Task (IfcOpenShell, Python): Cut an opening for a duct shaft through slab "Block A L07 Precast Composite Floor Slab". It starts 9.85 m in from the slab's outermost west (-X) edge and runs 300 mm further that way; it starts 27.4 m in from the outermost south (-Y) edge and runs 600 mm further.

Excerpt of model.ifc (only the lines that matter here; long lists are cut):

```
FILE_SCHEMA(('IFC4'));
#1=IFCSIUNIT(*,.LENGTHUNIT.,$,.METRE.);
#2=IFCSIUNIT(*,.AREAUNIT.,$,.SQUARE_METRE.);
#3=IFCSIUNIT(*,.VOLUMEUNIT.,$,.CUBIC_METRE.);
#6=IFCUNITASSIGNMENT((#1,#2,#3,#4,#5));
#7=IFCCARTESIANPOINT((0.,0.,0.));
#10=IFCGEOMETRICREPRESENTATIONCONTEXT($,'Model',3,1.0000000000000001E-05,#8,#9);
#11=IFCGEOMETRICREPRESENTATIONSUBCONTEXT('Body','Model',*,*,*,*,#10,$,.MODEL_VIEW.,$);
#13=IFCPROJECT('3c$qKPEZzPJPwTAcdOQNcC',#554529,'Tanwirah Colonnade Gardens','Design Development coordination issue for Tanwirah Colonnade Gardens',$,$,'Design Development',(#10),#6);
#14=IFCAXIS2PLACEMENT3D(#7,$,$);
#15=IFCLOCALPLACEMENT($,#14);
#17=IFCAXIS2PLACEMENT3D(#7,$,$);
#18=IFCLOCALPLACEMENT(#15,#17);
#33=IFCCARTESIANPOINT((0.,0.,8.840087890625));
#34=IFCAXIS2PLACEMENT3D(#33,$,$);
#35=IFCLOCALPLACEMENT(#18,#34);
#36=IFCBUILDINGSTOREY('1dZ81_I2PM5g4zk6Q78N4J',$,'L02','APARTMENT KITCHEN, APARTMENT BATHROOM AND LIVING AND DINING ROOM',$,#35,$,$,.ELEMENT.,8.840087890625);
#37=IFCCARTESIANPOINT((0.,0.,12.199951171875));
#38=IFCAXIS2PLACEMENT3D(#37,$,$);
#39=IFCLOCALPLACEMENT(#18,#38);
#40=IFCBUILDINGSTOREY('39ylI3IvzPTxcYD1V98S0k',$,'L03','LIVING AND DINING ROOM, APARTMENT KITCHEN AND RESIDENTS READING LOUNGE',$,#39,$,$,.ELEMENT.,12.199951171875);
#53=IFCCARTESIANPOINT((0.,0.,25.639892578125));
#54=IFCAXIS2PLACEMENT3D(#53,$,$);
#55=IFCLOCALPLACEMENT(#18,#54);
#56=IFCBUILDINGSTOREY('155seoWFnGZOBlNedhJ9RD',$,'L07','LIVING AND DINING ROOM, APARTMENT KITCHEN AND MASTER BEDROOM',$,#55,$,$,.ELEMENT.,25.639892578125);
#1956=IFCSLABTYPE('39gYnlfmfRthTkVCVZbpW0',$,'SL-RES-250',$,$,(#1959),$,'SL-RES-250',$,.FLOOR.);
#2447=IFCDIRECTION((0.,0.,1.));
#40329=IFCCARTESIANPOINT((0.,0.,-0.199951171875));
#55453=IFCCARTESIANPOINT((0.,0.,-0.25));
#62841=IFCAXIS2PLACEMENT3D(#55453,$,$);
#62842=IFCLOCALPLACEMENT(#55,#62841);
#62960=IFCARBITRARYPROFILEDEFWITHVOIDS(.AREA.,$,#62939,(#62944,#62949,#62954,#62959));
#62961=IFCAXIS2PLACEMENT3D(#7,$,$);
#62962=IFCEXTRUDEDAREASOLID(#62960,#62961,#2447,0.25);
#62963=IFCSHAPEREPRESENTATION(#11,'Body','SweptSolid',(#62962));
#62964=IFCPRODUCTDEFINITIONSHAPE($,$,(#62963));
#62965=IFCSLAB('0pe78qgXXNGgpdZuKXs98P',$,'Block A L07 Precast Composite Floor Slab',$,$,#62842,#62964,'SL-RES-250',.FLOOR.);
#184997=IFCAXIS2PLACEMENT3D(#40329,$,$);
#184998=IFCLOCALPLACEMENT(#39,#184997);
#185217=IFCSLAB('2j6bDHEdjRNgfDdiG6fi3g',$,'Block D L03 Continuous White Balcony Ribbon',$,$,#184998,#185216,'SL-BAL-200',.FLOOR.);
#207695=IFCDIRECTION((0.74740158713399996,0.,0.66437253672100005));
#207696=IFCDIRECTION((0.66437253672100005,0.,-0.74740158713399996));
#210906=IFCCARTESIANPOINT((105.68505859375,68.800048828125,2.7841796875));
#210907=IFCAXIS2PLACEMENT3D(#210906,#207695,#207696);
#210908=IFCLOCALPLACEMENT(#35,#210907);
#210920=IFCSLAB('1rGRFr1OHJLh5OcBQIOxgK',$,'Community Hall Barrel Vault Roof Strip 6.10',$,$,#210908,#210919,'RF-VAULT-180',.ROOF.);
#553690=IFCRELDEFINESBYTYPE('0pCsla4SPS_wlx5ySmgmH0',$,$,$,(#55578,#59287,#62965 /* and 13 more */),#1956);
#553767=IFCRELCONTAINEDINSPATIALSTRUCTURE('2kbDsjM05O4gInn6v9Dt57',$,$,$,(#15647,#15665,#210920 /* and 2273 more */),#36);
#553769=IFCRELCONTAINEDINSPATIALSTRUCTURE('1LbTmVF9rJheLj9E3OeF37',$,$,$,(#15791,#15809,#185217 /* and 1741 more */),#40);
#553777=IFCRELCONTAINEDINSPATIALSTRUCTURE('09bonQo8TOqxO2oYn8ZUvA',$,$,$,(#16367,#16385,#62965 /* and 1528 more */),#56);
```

```python
import numpy as np
import ifcopenshell
import ifcopenshell.api.feature
import ifcopenshell.api.geometry
import ifcopenshell.api.root
import ifcopenshell.geom
import ifcopenshell.util.placement
import ifcopenshell.util.representation
import ifcopenshell.util.shape
import ifcopenshell.util.unit

model = ifcopenshell.open("model.ifc")
unit_scale = ifcopenshell.util.unit.calculate_unit_scale(model)
settings = ifcopenshell.geom.settings()


def volume(element):
    """Net volume in cubic metres, openings subtracted."""
    shape = ifcopenshell.geom.create_shape(settings, element)
    return ifcopenshell.util.shape.get_volume(shape.geometry)


slab = model.by_id(62965)
before = volume(slab)

# Extent in the slab's own axes, in metres. The edges named are its -X and -Y sides.
slab_shape = ifcopenshell.geom.create_shape(settings, slab)
vertices = ifcopenshell.util.shape.get_vertices(slab_shape.geometry)
x_min, y_min, bottom = vertices.min(axis=0)
top = vertices[:, 2].max()

opening = ifcopenshell.api.root.create_entity(model, ifc_class="IfcOpeningElement", name="Duct shaft opening", predefined_type="OPENING")
context = ifcopenshell.util.representation.get_context(model, "Model", "Body", "MODEL_VIEW")
width, depth = 0.3, 0.6
outline = [(0.0, 0.0), (width, 0.0), (width, depth), (0.0, depth), (0.0, 0.0)]
# Overshoot both faces by 50 mm so the cut is clean.
shape = ifcopenshell.api.geometry.add_slab_representation(
    model, context=context, depth=top - bottom + 0.1, polyline=outline
)
ifcopenshell.api.geometry.assign_representation(model, product=opening, representation=shape)

matrix = ifcopenshell.util.placement.get_local_placement(slab.ObjectPlacement)
matrix[:, 3] = matrix @ np.append(np.array([x_min + 9.85, y_min + 27.4, bottom - 0.05]) / unit_scale, 1.0)
ifcopenshell.api.geometry.edit_object_placement(model, product=opening, matrix=matrix, is_si=False)
ifcopenshell.api.feature.add_feature(model, feature=opening, element=slab)

after = volume(slab)

print(f"slab volume {before:.3f} -> {after:.3f} m3")

model.write("model_v2.ifc")
```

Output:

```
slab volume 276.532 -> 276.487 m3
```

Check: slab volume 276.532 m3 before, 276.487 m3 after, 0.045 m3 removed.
